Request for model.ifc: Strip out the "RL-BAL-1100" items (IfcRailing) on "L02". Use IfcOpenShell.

First a look at what the model holds.

```python
import ifcopenshell
import ifcopenshell.util.element

model = ifcopenshell.open("model.ifc")
print(model.schema)
storey = next(s for s in model.by_type("IfcBuildingStorey") if s.Name == "L02")
railings = [e for e in ifcopenshell.util.element.get_decomposition(storey) if e.is_a("IfcRailing")]
seen = {}
for e in railings:
    element_type = ifcopenshell.util.element.get_type(e)
    name = element_type.Name if element_type not in (None, e) else None
    seen[name] = seen.get(name, 0) + 1
for name, count in sorted(seen.items(), key=str):
    print(count, "x", name)
```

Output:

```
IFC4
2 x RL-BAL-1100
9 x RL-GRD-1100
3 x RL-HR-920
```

```python
import ifcopenshell
import ifcopenshell.api.root
import ifcopenshell.util.element

model = ifcopenshell.open("model.ifc")

storey = next(s for s in model.by_type("IfcBuildingStorey") if s.Name == "L02")
railings = [e for e in ifcopenshell.util.element.get_decomposition(storey) if e.is_a("IfcRailing")]
targets = [e for e in railings if (t := ifcopenshell.util.element.get_type(e)) not in (None, e) and t.Name == "RL-BAL-1100"]

for e in targets:
    ifcopenshell.api.root.remove_product(model, product=e)
print(len(targets), "removed")

model.write("model_v2.ifc")
```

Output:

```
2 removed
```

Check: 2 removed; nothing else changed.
